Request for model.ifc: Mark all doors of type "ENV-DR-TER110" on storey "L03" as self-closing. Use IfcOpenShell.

First a look at what the model holds.

```python
import ifcopenshell
import ifcopenshell.util.element

model = ifcopenshell.open("model.ifc")
print(model.schema)
storey = next(s for s in model.by_type("IfcBuildingStorey") if s.Name == "L03")
doors = [e for e in ifcopenshell.util.element.get_decomposition(storey) if e.is_a("IfcDoor")]
seen = {}
for e in doors:
    element_type = ifcopenshell.util.element.get_type(e)
    key = (element_type.Name if element_type != e and element_type else None, ifcopenshell.util.element.get_pset(e, "Pset_DoorCommon", "SelfClosing"))
    seen[key] = seen.get(key, 0) + 1
for (name, value), count in sorted(seen.items(), key=str):
    print(count, "x", name, "|", value)
```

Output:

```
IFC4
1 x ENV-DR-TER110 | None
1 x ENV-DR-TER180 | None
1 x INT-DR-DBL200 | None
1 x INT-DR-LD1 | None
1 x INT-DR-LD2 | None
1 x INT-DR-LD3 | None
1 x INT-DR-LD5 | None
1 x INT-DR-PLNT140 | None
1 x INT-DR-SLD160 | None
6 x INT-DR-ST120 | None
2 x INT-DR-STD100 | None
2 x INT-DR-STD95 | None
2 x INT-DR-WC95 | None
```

```python
import ifcopenshell
import ifcopenshell.api.pset
import ifcopenshell.util.element

model = ifcopenshell.open("model.ifc")

storey = next(s for s in model.by_type("IfcBuildingStorey") if s.Name == "L03")
doors = [e for e in ifcopenshell.util.element.get_decomposition(storey) if e.is_a("IfcDoor")]

count = 0
for e in doors:
    element_type = ifcopenshell.util.element.get_type(e)
    if element_type in (None, e) or element_type.Name != "ENV-DR-TER110":
        continue
    # add_pset returns the element's existing set when there is one.
    pset = ifcopenshell.api.pset.add_pset(model, product=e, name="Pset_DoorCommon")
    ifcopenshell.api.pset.edit_pset(model, pset=pset, properties={"SelfClosing": True})
    count += 1

print(count, "doors updated")

model.write("model_v2.ifc")
```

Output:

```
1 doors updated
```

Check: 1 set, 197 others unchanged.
